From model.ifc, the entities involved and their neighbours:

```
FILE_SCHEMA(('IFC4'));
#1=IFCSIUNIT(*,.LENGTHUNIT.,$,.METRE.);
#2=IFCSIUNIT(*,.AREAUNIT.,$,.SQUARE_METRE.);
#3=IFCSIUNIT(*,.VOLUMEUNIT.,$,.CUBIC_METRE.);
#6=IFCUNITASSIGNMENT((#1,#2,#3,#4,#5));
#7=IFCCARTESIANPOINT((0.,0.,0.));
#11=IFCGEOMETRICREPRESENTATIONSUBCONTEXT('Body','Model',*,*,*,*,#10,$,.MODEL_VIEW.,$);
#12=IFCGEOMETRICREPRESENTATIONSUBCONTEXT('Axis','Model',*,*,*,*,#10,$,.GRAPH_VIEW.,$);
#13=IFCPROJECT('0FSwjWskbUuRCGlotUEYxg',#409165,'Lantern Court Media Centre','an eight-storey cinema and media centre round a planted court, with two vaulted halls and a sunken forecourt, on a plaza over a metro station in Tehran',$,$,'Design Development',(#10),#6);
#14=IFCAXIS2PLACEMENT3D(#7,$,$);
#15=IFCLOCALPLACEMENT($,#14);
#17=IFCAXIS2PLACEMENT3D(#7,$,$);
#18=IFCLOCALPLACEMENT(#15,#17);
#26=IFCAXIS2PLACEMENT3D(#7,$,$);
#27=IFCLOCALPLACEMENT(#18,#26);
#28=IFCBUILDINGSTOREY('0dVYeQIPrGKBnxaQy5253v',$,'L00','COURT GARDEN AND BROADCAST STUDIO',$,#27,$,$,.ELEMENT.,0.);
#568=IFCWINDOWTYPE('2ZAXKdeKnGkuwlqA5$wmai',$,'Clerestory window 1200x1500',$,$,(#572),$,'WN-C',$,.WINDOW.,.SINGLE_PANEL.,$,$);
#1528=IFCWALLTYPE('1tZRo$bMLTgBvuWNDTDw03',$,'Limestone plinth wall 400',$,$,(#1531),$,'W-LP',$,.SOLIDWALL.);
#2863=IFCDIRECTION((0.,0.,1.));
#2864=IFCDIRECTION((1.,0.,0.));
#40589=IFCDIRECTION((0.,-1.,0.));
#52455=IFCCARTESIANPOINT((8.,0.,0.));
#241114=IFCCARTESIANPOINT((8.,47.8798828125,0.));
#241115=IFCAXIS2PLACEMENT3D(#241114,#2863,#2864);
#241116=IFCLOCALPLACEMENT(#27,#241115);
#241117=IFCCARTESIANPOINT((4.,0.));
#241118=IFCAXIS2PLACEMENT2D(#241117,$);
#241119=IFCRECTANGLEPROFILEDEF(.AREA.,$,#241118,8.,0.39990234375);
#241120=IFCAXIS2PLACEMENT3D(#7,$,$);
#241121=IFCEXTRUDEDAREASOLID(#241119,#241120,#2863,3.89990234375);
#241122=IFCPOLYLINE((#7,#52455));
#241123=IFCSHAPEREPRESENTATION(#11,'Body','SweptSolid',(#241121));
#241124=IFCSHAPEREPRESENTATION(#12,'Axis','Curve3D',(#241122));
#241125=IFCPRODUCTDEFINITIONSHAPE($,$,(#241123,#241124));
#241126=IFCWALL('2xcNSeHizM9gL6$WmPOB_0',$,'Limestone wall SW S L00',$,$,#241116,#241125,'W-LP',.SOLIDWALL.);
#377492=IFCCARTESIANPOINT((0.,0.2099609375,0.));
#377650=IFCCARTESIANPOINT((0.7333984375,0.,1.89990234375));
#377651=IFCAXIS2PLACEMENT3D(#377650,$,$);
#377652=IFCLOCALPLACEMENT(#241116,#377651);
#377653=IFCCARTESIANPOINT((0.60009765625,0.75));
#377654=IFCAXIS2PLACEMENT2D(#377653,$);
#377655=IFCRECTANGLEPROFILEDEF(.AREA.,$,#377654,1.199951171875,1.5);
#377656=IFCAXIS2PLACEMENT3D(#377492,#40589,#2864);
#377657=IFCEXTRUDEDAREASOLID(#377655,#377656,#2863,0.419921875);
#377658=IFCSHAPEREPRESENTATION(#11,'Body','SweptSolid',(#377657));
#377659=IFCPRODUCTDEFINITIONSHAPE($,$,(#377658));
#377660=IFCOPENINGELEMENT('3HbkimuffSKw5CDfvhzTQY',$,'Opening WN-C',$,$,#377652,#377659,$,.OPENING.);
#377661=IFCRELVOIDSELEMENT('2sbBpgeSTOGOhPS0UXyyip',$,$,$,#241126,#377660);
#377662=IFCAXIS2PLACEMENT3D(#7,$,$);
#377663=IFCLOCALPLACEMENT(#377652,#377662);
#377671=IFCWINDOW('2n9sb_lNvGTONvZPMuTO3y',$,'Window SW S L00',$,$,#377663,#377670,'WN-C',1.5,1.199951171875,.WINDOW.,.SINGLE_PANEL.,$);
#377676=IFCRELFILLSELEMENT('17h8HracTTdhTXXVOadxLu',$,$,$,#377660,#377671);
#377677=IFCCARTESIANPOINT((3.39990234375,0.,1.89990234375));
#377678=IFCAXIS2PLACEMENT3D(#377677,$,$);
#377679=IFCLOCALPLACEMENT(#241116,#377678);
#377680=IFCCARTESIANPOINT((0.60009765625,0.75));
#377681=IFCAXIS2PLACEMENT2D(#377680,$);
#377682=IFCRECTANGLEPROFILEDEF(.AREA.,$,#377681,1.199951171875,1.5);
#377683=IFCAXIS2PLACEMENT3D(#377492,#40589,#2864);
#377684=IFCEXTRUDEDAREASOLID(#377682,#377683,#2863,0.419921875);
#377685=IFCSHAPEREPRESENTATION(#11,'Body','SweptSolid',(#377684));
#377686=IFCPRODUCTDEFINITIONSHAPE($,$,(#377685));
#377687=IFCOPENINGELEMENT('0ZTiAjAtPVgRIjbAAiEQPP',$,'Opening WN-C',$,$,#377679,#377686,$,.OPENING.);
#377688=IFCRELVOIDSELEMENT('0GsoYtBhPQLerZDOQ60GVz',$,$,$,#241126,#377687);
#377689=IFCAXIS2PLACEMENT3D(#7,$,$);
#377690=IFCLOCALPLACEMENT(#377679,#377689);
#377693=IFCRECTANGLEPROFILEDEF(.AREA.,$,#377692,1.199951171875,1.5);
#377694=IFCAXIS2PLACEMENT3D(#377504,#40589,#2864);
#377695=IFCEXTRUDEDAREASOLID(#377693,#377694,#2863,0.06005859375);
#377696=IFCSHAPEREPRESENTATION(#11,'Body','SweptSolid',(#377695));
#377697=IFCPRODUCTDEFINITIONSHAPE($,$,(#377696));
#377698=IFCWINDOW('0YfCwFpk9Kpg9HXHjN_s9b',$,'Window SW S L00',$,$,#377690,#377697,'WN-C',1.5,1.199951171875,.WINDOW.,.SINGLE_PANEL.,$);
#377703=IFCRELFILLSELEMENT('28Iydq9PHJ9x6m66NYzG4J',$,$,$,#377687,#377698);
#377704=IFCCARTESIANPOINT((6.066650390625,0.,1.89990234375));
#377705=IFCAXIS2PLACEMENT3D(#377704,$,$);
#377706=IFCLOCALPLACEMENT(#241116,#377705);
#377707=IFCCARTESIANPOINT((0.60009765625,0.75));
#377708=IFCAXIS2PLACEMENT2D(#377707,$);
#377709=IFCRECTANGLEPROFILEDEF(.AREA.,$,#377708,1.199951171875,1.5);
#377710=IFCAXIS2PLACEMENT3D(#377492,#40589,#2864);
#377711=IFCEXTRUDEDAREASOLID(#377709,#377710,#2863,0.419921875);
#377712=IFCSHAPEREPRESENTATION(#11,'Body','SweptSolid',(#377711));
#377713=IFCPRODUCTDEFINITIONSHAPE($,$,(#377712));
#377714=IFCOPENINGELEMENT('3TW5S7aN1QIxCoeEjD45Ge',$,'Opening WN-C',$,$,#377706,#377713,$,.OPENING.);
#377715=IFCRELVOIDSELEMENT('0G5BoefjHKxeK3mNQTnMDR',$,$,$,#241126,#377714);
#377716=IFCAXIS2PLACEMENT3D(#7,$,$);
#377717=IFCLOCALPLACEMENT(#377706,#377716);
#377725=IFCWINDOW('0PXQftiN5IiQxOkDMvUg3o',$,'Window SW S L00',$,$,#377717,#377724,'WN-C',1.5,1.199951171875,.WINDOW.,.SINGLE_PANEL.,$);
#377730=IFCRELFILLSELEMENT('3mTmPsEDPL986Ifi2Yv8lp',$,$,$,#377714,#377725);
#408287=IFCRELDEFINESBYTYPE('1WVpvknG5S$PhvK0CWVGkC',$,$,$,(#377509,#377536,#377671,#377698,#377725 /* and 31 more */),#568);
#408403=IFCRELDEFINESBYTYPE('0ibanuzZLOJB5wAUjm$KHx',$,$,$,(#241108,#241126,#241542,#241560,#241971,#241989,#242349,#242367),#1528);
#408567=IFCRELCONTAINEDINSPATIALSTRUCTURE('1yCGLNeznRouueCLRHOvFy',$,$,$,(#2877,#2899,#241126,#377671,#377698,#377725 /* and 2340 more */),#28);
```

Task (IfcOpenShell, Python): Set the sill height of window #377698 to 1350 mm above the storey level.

```python
import numpy as np
import ifcopenshell
import ifcopenshell.api.geometry
import ifcopenshell.geom
import ifcopenshell.util.element
import ifcopenshell.util.placement
import ifcopenshell.util.shape
import ifcopenshell.util.unit

model = ifcopenshell.open("model.ifc")
unit_scale = ifcopenshell.util.unit.calculate_unit_scale(model)

window = model.by_id(377698)
opening = window.FillsVoids[0].RelatingOpeningElement
storey = ifcopenshell.util.element.get_container(window, ifc_class="IfcBuildingStorey")
level = ifcopenshell.util.placement.get_local_placement(storey.ObjectPlacement)[2, 3]

# The opening's origin need not be at the sill, so measure its lowest point.
shape = ifcopenshell.geom.create_shape(ifcopenshell.geom.settings(), opening)
bottom = ifcopenshell.util.shape.get_shape_bottom_elevation(shape, shape.geometry) / unit_scale
dz = level + 1.35 / unit_scale - bottom

shift = np.array([0.0, 0.0, dz])
# The window is placed relative to its opening, so it follows when the opening moves.
matrix = ifcopenshell.util.placement.get_local_placement(opening.ObjectPlacement)
matrix[:3, 3] += shift
ifcopenshell.api.geometry.edit_object_placement(
    model, product=opening, matrix=matrix, is_si=False, should_transform_children=True
)

print(f"moved by {dz * unit_scale:+.3f} m")

model.write("model_updated.ifc")
```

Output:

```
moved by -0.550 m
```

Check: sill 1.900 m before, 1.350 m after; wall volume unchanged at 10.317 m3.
